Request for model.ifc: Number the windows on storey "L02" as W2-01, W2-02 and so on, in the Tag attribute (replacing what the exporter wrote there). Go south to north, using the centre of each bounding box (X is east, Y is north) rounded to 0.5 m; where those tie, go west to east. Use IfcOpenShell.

First a look at what the model holds.

```python
import ifcopenshell
import ifcopenshell.util.element
import ifcopenshell.util.placement

model = ifcopenshell.open("model.ifc")
print(model.schema)
storey = next(s for s in model.by_type("IfcBuildingStorey") if s.Name == "L02")
windows = [e for e in ifcopenshell.util.element.get_decomposition(storey) if e.is_a("IfcWindow")]
for e in sorted(windows, key=lambda e: e.id()):
    origin = ifcopenshell.util.placement.get_local_placement(e.ObjectPlacement)[:3, 3]
    print(e.id(), e.Tag, e.Name, origin.round(2) + 0.0, sep=" | ")
```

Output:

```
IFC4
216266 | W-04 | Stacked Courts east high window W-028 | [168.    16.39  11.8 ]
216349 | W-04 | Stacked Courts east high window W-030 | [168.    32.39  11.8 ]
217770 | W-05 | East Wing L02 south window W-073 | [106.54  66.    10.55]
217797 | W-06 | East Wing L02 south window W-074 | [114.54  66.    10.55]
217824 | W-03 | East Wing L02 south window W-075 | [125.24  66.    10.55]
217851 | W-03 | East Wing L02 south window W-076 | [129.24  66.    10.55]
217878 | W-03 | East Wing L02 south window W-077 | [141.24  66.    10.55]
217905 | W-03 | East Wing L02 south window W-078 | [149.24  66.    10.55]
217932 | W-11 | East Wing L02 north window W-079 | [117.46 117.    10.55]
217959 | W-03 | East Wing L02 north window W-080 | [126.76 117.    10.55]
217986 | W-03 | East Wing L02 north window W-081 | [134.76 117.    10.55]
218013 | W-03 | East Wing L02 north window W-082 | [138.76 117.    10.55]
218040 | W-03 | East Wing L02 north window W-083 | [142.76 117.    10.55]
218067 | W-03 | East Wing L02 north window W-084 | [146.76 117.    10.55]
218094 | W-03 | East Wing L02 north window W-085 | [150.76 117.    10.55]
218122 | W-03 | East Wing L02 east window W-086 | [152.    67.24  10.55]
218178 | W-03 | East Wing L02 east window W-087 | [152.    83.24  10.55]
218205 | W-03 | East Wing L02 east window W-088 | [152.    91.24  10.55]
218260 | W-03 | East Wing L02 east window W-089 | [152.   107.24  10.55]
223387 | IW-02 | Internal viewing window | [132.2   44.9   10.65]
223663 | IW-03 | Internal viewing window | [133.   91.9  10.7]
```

```python
import ifcopenshell
import ifcopenshell.geom
import ifcopenshell.util.element
import ifcopenshell.util.shape

model = ifcopenshell.open("model.ifc")
settings = ifcopenshell.geom.settings()
settings.set("use-world-coords", True)


def centre(element):
    shape = ifcopenshell.geom.create_shape(settings, element)
    return ifcopenshell.util.shape.get_bbox_centroid(shape.geometry)


storey = next(s for s in model.by_type("IfcBuildingStorey") if s.Name == "L02")
windows = [e for e in ifcopenshell.util.element.get_decomposition(storey) if e.is_a("IfcWindow")]

# Insertion points can sit at a corner or the storey origin, so sort by the geometry (in metres).
centres = {e: centre(e) for e in windows}
windows.sort(key=lambda e: (round(centres[e][1] / 0.5), centres[e][0]))

for i, e in enumerate(windows, start=1):
    number = f"W2-{i:02d}"
    e.Tag = number
    print(e.id(), number)

model.write("model_v2.ifc")
```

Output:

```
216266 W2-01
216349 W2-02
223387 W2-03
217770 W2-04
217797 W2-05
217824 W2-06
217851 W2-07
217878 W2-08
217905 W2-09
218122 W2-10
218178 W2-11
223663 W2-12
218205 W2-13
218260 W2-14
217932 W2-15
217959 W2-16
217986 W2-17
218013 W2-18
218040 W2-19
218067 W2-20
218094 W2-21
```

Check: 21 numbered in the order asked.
